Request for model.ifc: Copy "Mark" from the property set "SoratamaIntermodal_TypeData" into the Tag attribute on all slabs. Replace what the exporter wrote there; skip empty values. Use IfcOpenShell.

First a look at what the model holds.

```python
import ifcopenshell
import ifcopenshell.util.element

model = ifcopenshell.open("model.ifc")
print(model.schema)
slabs = model.by_type("IfcSlab")
print(len(slabs), "slabs")
for e in slabs[:8]:
    source = ifcopenshell.util.element.get_pset(e, "SoratamaIntermodal_TypeData", "Mark")
    target = e.Tag
    print(e.id(), repr(source), repr(target), sep=" | ")
```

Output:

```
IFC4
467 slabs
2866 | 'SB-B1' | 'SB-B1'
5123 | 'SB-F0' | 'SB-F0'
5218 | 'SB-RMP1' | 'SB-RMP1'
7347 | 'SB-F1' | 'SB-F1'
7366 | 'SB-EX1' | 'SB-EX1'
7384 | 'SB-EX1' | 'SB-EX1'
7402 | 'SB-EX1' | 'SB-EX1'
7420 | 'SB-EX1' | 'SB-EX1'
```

```python
import ifcopenshell
import ifcopenshell.util.element

model = ifcopenshell.open("model.ifc")

count = 0
for e in model.by_type("IfcSlab"):
    value = ifcopenshell.util.element.get_pset(e, "SoratamaIntermodal_TypeData", "Mark")
    current = e.Tag
    if not value or not value.strip() or current == value:
        continue
    e.Tag = value
    count += 1

print(count, "slabs updated")

model.write("model_rev.ifc")
```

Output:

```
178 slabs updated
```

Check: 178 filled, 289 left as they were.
